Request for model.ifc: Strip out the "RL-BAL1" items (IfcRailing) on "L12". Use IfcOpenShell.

First a look at what the model holds.

```python
import ifcopenshell
import ifcopenshell.util.element

model = ifcopenshell.open("model.ifc")
print(model.schema)
storey = next(s for s in model.by_type("IfcBuildingStorey") if s.Name == "L12")
railings = [e for e in ifcopenshell.util.element.get_decomposition(storey) if e.is_a("IfcRailing")]
seen = {}
for e in railings:
    element_type = ifcopenshell.util.element.get_type(e)
    name = element_type.Name if element_type not in (None, e) else None
    seen[name] = seen.get(name, 0) + 1
for name, count in sorted(seen.items(), key=str):
    print(count, "x", name)
```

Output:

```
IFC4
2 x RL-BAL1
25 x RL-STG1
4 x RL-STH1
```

```python
import ifcopenshell
import ifcopenshell.api.root
import ifcopenshell.util.element

model = ifcopenshell.open("model.ifc")

storey = next(s for s in model.by_type("IfcBuildingStorey") if s.Name == "L12")
railings = [e for e in ifcopenshell.util.element.get_decomposition(storey) if e.is_a("IfcRailing")]
targets = [e for e in railings if (t := ifcopenshell.util.element.get_type(e)) not in (None, e) and t.Name == "RL-BAL1"]

for e in targets:
    ifcopenshell.api.root.remove_product(model, product=e)
print(len(targets), "removed")

model.write("model_rev.ifc")
```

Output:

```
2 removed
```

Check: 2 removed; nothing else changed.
